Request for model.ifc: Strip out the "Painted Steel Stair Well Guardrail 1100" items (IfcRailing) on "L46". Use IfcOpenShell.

First a look at what the model holds.

```python
import ifcopenshell
import ifcopenshell.util.element

model = ifcopenshell.open("model.ifc")
print(model.schema)
storey = next(s for s in model.by_type("IfcBuildingStorey") if s.Name == "L46")
railings = [e for e in ifcopenshell.util.element.get_decomposition(storey) if e.is_a("IfcRailing")]
seen = {}
for e in railings:
    element_type = ifcopenshell.util.element.get_type(e)
    name = element_type.Name if element_type not in (None, e) else None
    seen[name] = seen.get(name, 0) + 1
for name, count in sorted(seen.items(), key=str):
    print(count, "x", name)
```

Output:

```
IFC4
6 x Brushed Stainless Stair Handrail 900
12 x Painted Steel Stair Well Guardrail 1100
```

```python
import ifcopenshell
import ifcopenshell.api.root
import ifcopenshell.util.element

model = ifcopenshell.open("model.ifc")

storey = next(s for s in model.by_type("IfcBuildingStorey") if s.Name == "L46")
railings = [e for e in ifcopenshell.util.element.get_decomposition(storey) if e.is_a("IfcRailing")]
targets = [e for e in railings if (t := ifcopenshell.util.element.get_type(e)) not in (None, e) and t.Name == "Painted Steel Stair Well Guardrail 1100"]

for e in targets:
    ifcopenshell.api.root.remove_product(model, product=e)
print(len(targets), "removed")

model.write("model_v2.ifc")
```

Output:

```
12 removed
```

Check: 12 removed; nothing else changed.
